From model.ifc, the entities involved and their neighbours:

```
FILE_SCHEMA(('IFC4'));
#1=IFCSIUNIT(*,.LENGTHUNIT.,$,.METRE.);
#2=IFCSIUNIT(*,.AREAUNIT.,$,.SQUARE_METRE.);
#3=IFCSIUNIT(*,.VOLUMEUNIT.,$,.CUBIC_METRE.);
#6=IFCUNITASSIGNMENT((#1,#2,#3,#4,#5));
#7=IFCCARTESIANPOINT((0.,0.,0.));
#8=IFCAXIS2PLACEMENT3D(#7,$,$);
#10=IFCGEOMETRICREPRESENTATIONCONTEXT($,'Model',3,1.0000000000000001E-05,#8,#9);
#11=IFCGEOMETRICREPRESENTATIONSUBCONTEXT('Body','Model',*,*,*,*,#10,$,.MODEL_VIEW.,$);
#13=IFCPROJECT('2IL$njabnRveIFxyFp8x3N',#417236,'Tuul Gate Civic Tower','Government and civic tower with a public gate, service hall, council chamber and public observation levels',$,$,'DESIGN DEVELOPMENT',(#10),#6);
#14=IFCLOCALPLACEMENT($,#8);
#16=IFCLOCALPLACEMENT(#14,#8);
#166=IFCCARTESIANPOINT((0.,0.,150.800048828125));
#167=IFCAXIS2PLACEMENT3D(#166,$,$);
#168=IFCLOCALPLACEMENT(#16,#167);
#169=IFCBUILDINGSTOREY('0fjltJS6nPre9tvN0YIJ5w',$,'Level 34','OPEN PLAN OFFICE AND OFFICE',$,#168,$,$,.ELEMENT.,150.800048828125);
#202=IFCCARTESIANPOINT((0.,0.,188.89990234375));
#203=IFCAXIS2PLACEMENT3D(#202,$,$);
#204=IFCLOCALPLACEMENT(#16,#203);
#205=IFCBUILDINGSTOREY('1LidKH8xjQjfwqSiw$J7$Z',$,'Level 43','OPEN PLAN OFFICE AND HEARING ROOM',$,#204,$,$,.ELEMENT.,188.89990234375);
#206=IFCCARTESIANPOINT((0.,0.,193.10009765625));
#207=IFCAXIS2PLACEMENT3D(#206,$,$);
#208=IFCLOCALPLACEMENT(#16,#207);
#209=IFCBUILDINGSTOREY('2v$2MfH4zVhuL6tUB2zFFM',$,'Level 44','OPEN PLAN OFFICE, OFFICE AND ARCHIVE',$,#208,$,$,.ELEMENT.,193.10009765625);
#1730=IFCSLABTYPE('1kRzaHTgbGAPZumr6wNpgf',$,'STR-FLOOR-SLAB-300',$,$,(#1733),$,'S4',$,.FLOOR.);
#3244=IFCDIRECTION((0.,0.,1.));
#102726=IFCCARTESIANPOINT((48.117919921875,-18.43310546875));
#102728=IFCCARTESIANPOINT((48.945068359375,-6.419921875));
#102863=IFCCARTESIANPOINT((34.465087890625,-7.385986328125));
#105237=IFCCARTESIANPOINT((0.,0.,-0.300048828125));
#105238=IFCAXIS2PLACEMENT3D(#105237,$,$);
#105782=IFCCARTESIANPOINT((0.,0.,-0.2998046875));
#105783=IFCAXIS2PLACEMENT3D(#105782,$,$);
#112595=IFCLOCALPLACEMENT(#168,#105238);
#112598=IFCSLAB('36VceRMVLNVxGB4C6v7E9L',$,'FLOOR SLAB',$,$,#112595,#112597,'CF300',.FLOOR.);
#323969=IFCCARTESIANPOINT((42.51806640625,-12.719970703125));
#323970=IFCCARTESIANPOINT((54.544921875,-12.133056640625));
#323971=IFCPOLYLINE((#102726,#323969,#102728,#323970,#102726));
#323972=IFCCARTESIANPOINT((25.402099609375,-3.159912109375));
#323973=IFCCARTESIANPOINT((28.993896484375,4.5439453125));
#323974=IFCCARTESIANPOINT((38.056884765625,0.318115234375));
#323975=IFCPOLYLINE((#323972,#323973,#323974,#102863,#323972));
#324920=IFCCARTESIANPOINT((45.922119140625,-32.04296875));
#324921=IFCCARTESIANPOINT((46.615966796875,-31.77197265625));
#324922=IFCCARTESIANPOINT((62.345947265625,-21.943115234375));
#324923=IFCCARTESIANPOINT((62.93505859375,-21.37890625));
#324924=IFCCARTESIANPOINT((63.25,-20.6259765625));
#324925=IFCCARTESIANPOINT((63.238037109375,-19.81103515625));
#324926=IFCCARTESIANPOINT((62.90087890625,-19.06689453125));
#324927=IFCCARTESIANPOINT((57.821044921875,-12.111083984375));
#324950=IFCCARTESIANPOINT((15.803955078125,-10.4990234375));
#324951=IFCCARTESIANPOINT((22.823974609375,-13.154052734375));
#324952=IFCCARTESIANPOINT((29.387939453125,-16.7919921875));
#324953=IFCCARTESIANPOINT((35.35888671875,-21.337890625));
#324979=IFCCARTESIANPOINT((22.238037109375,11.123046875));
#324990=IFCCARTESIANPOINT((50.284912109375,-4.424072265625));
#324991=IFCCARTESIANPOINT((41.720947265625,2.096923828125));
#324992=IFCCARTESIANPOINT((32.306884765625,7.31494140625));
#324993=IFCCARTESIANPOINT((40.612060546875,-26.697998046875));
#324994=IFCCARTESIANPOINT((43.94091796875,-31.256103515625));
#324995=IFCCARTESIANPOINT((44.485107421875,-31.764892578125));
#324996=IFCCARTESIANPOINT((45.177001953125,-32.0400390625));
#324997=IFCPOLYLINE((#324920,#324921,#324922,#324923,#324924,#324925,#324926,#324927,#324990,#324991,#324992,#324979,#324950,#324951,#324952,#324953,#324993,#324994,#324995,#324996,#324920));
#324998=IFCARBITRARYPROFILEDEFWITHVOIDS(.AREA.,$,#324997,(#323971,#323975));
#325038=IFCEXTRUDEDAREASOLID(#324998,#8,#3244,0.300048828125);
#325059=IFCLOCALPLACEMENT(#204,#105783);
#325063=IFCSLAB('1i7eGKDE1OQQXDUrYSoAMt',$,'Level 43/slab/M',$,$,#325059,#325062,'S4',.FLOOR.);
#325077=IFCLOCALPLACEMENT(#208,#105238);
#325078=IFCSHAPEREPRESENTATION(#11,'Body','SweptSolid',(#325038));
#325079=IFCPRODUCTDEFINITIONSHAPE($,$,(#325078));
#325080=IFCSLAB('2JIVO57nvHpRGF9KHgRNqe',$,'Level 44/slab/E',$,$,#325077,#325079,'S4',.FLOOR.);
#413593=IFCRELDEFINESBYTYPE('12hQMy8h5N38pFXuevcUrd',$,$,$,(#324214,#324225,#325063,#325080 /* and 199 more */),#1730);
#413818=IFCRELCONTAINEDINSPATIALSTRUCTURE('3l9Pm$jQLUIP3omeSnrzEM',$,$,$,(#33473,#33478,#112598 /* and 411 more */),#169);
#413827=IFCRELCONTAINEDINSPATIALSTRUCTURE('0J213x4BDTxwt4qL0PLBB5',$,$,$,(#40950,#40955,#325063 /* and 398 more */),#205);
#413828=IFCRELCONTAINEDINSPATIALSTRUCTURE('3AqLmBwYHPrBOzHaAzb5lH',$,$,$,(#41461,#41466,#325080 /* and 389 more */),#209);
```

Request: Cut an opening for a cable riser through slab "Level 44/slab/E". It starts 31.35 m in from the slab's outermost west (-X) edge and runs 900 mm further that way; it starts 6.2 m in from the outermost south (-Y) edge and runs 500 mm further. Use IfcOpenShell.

```python
import numpy as np
import ifcopenshell
import ifcopenshell.api.feature
import ifcopenshell.api.geometry
import ifcopenshell.api.root
import ifcopenshell.geom
import ifcopenshell.util.placement
import ifcopenshell.util.representation
import ifcopenshell.util.shape
import ifcopenshell.util.unit

model = ifcopenshell.open("model.ifc")
unit_scale = ifcopenshell.util.unit.calculate_unit_scale(model)
settings = ifcopenshell.geom.settings()


def volume(element):
    """Net volume in cubic metres, openings subtracted."""
    shape = ifcopenshell.geom.create_shape(settings, element)
    return ifcopenshell.util.shape.get_volume(shape.geometry)


slab = model.by_guid("2JIVO57nvHpRGF9KHgRNqe")
before = volume(slab)

# Extent in the slab's own axes, in metres. The edges named are its -X and -Y sides.
slab_shape = ifcopenshell.geom.create_shape(settings, slab)
vertices = ifcopenshell.util.shape.get_vertices(slab_shape.geometry)
x_min, y_min, bottom = vertices.min(axis=0)
top = vertices[:, 2].max()

opening = ifcopenshell.api.root.create_entity(model, ifc_class="IfcOpeningElement", name="Cable riser opening", predefined_type="OPENING")
context = ifcopenshell.util.representation.get_context(model, "Model", "Body", "MODEL_VIEW")
width, depth = 0.9, 0.5
outline = [(0.0, 0.0), (width, 0.0), (width, depth), (0.0, depth), (0.0, 0.0)]
# Overshoot both faces by 50 mm so the cut is clean.
shape = ifcopenshell.api.geometry.add_slab_representation(
    model, context=context, depth=top - bottom + 0.1, polyline=outline
)
ifcopenshell.api.geometry.assign_representation(model, product=opening, representation=shape)

matrix = ifcopenshell.util.placement.get_local_placement(slab.ObjectPlacement)
matrix[:, 3] = matrix @ np.append(np.array([x_min + 31.35, y_min + 6.2, bottom - 0.05]) / unit_scale, 1.0)
ifcopenshell.api.geometry.edit_object_placement(model, product=opening, matrix=matrix, is_si=False)
ifcopenshell.api.feature.add_feature(model, feature=opening, element=slab)

after = volume(slab)

print(f"slab volume {before:.3f} -> {after:.3f} m3")

model.write("model_edited.ifc")
```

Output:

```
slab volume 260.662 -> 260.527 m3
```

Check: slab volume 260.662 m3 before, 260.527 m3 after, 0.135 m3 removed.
